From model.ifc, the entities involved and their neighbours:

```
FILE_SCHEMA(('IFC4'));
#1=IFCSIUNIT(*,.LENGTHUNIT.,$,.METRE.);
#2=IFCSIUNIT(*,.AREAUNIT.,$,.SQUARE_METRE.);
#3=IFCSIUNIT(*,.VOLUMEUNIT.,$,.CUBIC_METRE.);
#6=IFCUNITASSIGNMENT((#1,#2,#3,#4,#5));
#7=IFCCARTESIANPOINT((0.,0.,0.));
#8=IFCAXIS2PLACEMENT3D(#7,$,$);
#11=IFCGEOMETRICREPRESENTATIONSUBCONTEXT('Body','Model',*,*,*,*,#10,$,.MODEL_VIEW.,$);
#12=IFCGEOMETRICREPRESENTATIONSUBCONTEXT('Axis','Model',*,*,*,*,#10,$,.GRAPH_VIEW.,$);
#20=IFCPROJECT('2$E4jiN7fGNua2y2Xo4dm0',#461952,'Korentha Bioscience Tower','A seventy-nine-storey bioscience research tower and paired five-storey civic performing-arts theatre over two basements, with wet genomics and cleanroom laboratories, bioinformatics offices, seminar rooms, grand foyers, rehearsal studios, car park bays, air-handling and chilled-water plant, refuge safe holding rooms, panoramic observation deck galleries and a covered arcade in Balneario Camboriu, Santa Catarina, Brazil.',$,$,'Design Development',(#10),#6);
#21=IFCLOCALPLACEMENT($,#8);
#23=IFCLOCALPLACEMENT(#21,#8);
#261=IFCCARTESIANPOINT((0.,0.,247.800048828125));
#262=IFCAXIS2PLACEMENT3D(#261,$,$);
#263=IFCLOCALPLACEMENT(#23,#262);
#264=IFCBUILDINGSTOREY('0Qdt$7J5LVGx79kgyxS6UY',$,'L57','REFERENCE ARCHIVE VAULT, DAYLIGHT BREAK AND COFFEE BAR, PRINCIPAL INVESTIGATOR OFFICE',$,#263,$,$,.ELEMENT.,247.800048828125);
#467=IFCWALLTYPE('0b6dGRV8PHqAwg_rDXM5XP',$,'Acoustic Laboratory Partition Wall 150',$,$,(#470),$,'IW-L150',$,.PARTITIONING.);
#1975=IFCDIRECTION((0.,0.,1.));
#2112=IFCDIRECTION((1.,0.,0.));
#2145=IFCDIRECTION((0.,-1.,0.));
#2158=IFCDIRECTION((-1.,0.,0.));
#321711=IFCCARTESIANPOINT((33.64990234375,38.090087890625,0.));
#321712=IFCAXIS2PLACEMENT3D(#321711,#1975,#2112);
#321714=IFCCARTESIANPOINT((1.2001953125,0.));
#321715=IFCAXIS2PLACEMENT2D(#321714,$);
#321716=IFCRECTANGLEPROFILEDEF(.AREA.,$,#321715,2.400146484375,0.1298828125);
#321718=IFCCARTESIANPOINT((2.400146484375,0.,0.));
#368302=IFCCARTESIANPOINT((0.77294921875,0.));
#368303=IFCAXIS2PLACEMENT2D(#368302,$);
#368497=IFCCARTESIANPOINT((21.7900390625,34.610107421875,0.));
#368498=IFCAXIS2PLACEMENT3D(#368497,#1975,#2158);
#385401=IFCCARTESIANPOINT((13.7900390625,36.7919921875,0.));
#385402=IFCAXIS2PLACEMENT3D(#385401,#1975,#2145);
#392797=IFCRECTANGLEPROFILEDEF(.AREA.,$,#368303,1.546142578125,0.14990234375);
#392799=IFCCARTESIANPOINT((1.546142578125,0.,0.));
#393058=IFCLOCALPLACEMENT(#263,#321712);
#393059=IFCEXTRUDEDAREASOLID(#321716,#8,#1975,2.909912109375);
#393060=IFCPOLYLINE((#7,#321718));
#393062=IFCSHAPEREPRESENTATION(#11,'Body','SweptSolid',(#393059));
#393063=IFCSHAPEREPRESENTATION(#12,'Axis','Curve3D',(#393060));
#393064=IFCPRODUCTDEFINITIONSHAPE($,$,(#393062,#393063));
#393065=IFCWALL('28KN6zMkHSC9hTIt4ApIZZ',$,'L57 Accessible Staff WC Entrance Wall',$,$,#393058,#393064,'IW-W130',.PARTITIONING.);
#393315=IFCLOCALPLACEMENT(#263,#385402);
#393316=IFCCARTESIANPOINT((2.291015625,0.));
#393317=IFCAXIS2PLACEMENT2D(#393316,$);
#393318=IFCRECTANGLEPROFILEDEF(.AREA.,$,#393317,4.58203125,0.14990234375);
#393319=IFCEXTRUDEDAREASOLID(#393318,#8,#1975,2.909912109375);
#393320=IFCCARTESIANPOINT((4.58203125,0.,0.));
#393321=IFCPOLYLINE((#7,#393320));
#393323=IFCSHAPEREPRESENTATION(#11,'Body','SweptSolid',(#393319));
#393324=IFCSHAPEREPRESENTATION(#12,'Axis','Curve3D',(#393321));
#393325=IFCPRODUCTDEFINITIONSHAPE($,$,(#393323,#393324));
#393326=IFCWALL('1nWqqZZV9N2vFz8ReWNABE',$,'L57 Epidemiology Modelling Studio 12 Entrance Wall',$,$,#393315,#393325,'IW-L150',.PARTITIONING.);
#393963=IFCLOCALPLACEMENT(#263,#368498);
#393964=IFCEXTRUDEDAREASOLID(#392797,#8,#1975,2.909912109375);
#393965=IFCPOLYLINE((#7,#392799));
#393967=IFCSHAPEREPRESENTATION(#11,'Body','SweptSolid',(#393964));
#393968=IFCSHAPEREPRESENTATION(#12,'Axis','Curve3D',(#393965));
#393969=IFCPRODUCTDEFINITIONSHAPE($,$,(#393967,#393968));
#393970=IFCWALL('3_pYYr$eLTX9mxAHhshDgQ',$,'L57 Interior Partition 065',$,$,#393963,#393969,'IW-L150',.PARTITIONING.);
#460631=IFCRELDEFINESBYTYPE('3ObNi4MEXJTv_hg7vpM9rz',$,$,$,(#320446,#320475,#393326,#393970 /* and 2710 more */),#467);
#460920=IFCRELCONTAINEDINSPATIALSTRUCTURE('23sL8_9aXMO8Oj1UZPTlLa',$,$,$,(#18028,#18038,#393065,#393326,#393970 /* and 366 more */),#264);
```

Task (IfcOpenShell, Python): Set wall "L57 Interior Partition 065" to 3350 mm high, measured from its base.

```python
import ifcopenshell
import ifcopenshell.geom
import ifcopenshell.util.representation
import ifcopenshell.util.shape

model = ifcopenshell.open("model.ifc")
settings = ifcopenshell.geom.settings()


def volume(element):
    """Net volume in cubic metres, openings subtracted."""
    shape = ifcopenshell.geom.create_shape(settings, element)
    return ifcopenshell.util.shape.get_volume(shape.geometry)


wall = model.by_guid("3_pYYr$eLTX9mxAHhshDgQ")
before = volume(wall)

body = ifcopenshell.util.representation.get_representation(wall, "Model", "Body")
solid = body.Items[0]
old_height = solid.Depth
solid.Depth = 3.35
after = volume(wall)

print(f"height {old_height:g} -> {solid.Depth:g}, volume {before:.3f} -> {after:.3f} m3")

model.write("model_rev.ifc")
```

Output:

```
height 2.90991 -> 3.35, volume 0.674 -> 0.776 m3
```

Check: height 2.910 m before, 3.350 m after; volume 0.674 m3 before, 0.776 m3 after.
